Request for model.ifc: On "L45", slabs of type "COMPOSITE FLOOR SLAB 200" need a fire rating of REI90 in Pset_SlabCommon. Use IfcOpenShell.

First a look at what the model holds.

```python
import ifcopenshell
import ifcopenshell.util.element

model = ifcopenshell.open("model.ifc")
print(model.schema)
storey = next(s for s in model.by_type("IfcBuildingStorey") if s.Name == "L45")
slabs = [e for e in ifcopenshell.util.element.get_decomposition(storey) if e.is_a("IfcSlab")]
seen = {}
for e in slabs:
    element_type = ifcopenshell.util.element.get_type(e)
    key = (element_type.Name if element_type != e and element_type else None, ifcopenshell.util.element.get_pset(e, "Pset_SlabCommon", "FireRating"))
    seen[key] = seen.get(key, 0) + 1
for (name, value), count in sorted(seen.items(), key=str):
    print(count, "x", name, "|", value)
```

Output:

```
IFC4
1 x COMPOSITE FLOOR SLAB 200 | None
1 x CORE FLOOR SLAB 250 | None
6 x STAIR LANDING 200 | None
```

```python
import ifcopenshell
import ifcopenshell.api.pset
import ifcopenshell.util.element

model = ifcopenshell.open("model.ifc")

storey = next(s for s in model.by_type("IfcBuildingStorey") if s.Name == "L45")
slabs = [e for e in ifcopenshell.util.element.get_decomposition(storey) if e.is_a("IfcSlab")]

count = 0
for e in slabs:
    element_type = ifcopenshell.util.element.get_type(e)
    if element_type in (None, e) or element_type.Name != "COMPOSITE FLOOR SLAB 200":
        continue
    found = ifcopenshell.util.element.get_pset(e, "Pset_SlabCommon", should_inherit=False)
    if found:
        pset = model.by_id(found["id"])
        if len(ifcopenshell.util.element.get_elements_by_pset(pset)) > 1:
            pset = ifcopenshell.api.pset.unshare_pset(model, products=[e], pset=pset)[0]
    else:
        pset = ifcopenshell.api.pset.add_pset(model, product=e, name="Pset_SlabCommon")
    ifcopenshell.api.pset.edit_pset(model, pset=pset, properties={"FireRating": "REI90"})
    count += 1

print(count, "slabs updated")

model.write("model_updated.ifc")
```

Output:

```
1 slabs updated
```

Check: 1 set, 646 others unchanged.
